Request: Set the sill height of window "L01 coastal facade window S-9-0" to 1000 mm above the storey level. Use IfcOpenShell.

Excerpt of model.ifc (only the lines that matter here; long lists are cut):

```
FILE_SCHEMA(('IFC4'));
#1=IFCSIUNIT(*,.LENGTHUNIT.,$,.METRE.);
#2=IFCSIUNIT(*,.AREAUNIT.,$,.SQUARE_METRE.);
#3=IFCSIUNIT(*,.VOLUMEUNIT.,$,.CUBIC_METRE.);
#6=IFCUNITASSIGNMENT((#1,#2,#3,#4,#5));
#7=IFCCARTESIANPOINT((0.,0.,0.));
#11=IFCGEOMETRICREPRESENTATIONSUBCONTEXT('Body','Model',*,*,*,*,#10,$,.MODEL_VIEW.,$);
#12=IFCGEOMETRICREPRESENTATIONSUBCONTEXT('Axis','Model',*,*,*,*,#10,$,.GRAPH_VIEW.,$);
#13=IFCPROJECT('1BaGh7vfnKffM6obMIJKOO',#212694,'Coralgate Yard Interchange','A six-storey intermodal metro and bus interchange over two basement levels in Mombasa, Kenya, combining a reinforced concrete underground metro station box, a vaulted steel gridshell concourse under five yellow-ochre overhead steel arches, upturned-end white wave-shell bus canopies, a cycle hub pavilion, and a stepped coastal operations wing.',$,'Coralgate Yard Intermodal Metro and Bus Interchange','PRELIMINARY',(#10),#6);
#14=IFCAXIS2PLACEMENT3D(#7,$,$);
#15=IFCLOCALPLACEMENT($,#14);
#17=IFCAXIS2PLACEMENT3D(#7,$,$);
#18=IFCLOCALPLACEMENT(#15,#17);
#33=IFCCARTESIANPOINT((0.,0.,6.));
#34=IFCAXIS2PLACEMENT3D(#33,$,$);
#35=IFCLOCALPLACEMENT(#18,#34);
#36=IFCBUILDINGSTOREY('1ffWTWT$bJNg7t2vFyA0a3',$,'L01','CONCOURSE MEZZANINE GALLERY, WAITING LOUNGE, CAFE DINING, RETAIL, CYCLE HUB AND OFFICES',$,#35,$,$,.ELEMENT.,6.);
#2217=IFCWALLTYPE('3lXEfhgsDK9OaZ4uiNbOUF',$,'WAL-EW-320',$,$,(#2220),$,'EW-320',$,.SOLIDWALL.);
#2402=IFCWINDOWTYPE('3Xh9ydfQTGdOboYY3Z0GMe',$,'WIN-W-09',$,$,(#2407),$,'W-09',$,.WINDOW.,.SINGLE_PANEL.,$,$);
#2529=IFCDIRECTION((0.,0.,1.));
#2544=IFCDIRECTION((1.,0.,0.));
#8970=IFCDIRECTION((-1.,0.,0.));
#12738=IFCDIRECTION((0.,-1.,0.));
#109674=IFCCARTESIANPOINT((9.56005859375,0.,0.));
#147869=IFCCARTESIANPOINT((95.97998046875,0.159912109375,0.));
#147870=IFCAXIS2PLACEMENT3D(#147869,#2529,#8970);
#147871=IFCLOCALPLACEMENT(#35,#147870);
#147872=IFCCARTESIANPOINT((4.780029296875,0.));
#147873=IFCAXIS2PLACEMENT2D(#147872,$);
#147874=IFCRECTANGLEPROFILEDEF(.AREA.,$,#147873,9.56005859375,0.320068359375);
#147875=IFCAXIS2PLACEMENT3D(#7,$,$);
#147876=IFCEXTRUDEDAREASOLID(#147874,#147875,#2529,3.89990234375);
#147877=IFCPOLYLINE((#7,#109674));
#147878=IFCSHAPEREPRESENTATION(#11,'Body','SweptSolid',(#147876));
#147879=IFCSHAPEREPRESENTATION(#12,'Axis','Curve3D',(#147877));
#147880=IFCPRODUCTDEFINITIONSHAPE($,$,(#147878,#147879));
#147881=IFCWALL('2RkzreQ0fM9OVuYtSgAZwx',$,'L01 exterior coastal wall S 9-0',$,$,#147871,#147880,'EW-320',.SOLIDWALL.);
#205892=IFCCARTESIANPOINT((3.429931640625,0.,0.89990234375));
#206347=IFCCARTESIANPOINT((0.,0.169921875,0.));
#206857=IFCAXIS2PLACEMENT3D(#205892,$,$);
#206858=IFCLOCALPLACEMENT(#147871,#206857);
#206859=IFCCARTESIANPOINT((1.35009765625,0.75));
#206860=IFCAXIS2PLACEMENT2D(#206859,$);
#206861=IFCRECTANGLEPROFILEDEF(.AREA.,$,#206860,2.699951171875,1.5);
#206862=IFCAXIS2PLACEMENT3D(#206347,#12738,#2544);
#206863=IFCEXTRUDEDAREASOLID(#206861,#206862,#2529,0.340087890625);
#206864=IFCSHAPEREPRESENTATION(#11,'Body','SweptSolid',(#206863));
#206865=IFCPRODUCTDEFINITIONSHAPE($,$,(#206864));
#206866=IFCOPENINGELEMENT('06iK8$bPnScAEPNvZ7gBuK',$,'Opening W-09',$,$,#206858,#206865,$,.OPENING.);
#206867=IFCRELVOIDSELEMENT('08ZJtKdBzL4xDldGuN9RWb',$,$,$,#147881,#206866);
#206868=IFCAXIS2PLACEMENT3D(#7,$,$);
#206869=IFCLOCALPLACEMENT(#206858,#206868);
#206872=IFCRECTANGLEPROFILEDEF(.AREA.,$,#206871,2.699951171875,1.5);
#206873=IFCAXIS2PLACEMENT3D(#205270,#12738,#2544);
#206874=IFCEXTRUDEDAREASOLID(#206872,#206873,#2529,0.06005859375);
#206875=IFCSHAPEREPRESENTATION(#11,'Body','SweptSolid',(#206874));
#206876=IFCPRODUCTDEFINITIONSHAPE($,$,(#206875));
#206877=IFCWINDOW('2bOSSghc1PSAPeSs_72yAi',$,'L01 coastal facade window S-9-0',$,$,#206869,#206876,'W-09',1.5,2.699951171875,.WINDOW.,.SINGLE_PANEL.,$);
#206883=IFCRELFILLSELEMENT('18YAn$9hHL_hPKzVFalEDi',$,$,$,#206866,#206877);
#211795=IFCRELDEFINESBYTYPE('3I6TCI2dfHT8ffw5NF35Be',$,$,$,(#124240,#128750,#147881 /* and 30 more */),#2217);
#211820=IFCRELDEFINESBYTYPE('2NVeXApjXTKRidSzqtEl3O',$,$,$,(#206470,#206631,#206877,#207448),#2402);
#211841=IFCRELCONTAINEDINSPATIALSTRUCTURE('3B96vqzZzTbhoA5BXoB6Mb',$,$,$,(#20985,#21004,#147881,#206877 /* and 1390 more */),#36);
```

```python
import numpy as np
import ifcopenshell
import ifcopenshell.api.geometry
import ifcopenshell.geom
import ifcopenshell.util.element
import ifcopenshell.util.placement
import ifcopenshell.util.shape
import ifcopenshell.util.unit

model = ifcopenshell.open("model.ifc")
unit_scale = ifcopenshell.util.unit.calculate_unit_scale(model)

window = model.by_id(206877)
opening = window.FillsVoids[0].RelatingOpeningElement
storey = ifcopenshell.util.element.get_container(window, ifc_class="IfcBuildingStorey")
level = ifcopenshell.util.placement.get_local_placement(storey.ObjectPlacement)[2, 3]

# The opening's origin need not be at the sill, so measure its lowest point.
shape = ifcopenshell.geom.create_shape(ifcopenshell.geom.settings(), opening)
bottom = ifcopenshell.util.shape.get_shape_bottom_elevation(shape, shape.geometry) / unit_scale
dz = level + 1.0 - bottom

shift = np.array([0.0, 0.0, dz])
# The window is placed relative to its opening, so it follows when the opening moves.
matrix = ifcopenshell.util.placement.get_local_placement(opening.ObjectPlacement)
matrix[:3, 3] += shift
ifcopenshell.api.geometry.edit_object_placement(
    model, product=opening, matrix=matrix, is_si=False, should_transform_children=True
)

print(f"moved by {dz * unit_scale:+.3f} m")

model.write("model_edited.ifc")
```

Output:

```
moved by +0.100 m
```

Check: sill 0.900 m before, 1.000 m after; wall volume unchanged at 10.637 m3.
